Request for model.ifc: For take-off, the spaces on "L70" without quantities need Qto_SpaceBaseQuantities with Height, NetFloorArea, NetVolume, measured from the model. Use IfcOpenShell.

First a look at what the model holds.

```python
import ifcopenshell
import ifcopenshell.util.element
import ifcopenshell.util.unit

model = ifcopenshell.open("model.ifc")
print(model.schema)
for unit_type in ("LENGTHUNIT", "AREAUNIT", "VOLUMEUNIT"):
    print(unit_type, ifcopenshell.util.unit.calculate_unit_scale(model, unit_type))
storey = next(s for s in model.by_type("IfcBuildingStorey") if s.Name == "L70")
spaces = [e for e in ifcopenshell.util.element.get_decomposition(storey) if e.is_a("IfcSpace")]
for e in sorted(spaces, key=lambda e: e.id()):
    print(e.id(), e.is_a(), e.Name, list(ifcopenshell.util.element.get_psets(e, qtos_only=True)), sep=" | ")
```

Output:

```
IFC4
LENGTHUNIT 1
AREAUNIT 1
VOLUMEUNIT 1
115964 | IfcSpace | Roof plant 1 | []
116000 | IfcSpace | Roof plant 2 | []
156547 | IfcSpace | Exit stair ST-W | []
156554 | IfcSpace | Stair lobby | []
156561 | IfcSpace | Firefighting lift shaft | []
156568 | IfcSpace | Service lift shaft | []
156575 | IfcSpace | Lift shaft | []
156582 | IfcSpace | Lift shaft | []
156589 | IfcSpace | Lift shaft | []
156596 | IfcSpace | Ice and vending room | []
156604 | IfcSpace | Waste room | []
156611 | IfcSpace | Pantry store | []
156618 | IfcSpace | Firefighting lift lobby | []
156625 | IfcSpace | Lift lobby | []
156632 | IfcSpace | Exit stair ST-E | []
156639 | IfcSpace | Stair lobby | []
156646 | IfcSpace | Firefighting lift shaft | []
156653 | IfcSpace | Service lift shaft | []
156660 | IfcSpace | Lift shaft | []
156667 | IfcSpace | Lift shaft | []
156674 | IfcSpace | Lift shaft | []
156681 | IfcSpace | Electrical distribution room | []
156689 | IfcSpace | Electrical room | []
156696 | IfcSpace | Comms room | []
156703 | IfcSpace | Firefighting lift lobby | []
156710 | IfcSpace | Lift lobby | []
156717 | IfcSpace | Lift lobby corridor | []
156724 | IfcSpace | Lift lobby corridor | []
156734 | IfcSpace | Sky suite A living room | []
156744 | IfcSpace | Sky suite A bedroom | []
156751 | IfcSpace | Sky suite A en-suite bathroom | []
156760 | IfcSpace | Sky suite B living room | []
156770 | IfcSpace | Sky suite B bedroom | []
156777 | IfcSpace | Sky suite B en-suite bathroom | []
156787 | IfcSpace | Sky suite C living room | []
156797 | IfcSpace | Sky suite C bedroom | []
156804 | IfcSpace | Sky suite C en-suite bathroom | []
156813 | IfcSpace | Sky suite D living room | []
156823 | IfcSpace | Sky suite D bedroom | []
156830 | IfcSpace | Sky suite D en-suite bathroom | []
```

```python
import ifcopenshell
import ifcopenshell.api.pset
import ifcopenshell.geom
import ifcopenshell.util.element
import ifcopenshell.util.shape
import ifcopenshell.util.unit

model = ifcopenshell.open("model.ifc")
unit_scale = ifcopenshell.util.unit.calculate_unit_scale(model)
area_scale = ifcopenshell.util.unit.calculate_unit_scale(model, "AREAUNIT")
volume_scale = ifcopenshell.util.unit.calculate_unit_scale(model, "VOLUMEUNIT")
settings = ifcopenshell.geom.settings()

storey = next(s for s in model.by_type("IfcBuildingStorey") if s.Name == "L70")
spaces = [e for e in ifcopenshell.util.element.get_decomposition(storey) if e.is_a("IfcSpace")]

for e in sorted(spaces, key=lambda e: e.id()):
    if ifcopenshell.util.element.get_psets(e, qtos_only=True, should_inherit=False):
        continue
    # Geometry comes back in metres, in the element's own axes.
    shape = ifcopenshell.geom.create_shape(settings, e)
    values = {
        "Height": ifcopenshell.util.shape.get_z(shape.geometry) / unit_scale,
        "NetFloorArea": ifcopenshell.util.shape.get_footprint_area(shape.geometry) / area_scale,
        "NetVolume": ifcopenshell.util.shape.get_volume(shape.geometry) / volume_scale,
    }
    qto = ifcopenshell.api.pset.add_qto(model, product=e, name="Qto_SpaceBaseQuantities")
    ifcopenshell.api.pset.edit_qto(model, qto=qto, properties=values)
    print(e.id(), {k: round(v, 3) for k, v in values.items()})

model.write("model-out.ifc")
```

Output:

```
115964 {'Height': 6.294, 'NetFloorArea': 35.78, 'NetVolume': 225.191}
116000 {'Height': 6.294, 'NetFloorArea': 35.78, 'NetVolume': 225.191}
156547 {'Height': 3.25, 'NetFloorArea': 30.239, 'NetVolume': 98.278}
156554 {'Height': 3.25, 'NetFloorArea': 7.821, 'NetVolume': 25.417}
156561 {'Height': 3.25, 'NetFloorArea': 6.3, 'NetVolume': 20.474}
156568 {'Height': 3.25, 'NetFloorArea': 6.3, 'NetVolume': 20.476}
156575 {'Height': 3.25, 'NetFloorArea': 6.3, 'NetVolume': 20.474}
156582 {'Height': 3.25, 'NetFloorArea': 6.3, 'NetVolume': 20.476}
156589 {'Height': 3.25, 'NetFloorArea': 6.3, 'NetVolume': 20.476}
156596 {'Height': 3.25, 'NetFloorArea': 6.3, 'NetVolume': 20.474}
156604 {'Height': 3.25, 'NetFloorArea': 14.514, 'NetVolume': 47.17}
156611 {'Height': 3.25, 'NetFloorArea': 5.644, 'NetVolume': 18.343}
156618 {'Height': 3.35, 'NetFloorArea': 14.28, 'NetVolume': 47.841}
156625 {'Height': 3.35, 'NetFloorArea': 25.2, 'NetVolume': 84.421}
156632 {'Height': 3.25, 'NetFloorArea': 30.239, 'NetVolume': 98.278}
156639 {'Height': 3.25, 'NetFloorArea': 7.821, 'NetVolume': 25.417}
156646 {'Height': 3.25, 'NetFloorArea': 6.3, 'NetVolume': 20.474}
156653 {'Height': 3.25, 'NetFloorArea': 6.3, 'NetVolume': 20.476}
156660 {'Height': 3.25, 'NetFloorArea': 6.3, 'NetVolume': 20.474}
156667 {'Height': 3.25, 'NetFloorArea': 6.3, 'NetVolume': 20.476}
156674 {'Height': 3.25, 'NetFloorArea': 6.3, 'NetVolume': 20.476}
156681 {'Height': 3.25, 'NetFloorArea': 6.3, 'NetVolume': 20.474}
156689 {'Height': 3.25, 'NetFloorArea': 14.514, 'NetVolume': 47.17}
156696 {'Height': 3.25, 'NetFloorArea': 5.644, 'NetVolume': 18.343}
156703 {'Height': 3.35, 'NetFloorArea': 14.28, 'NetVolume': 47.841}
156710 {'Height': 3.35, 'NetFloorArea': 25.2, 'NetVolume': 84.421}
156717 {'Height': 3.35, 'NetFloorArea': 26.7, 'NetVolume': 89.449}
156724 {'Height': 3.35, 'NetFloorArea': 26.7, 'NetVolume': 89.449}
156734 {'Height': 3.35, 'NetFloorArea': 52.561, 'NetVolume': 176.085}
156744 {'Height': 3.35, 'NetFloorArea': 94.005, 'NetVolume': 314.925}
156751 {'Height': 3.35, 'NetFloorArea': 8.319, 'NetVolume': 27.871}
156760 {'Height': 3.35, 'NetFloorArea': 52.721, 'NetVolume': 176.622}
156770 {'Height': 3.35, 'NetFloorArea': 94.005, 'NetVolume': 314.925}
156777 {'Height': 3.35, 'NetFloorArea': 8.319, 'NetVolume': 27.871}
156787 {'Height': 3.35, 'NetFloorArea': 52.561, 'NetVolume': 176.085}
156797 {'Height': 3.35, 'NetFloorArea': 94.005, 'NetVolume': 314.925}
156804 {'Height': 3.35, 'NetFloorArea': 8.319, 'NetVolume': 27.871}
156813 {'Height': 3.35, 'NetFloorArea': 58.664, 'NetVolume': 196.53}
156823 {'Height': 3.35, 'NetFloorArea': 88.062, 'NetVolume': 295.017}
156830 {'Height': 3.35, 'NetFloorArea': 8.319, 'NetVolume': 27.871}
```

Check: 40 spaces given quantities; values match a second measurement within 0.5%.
